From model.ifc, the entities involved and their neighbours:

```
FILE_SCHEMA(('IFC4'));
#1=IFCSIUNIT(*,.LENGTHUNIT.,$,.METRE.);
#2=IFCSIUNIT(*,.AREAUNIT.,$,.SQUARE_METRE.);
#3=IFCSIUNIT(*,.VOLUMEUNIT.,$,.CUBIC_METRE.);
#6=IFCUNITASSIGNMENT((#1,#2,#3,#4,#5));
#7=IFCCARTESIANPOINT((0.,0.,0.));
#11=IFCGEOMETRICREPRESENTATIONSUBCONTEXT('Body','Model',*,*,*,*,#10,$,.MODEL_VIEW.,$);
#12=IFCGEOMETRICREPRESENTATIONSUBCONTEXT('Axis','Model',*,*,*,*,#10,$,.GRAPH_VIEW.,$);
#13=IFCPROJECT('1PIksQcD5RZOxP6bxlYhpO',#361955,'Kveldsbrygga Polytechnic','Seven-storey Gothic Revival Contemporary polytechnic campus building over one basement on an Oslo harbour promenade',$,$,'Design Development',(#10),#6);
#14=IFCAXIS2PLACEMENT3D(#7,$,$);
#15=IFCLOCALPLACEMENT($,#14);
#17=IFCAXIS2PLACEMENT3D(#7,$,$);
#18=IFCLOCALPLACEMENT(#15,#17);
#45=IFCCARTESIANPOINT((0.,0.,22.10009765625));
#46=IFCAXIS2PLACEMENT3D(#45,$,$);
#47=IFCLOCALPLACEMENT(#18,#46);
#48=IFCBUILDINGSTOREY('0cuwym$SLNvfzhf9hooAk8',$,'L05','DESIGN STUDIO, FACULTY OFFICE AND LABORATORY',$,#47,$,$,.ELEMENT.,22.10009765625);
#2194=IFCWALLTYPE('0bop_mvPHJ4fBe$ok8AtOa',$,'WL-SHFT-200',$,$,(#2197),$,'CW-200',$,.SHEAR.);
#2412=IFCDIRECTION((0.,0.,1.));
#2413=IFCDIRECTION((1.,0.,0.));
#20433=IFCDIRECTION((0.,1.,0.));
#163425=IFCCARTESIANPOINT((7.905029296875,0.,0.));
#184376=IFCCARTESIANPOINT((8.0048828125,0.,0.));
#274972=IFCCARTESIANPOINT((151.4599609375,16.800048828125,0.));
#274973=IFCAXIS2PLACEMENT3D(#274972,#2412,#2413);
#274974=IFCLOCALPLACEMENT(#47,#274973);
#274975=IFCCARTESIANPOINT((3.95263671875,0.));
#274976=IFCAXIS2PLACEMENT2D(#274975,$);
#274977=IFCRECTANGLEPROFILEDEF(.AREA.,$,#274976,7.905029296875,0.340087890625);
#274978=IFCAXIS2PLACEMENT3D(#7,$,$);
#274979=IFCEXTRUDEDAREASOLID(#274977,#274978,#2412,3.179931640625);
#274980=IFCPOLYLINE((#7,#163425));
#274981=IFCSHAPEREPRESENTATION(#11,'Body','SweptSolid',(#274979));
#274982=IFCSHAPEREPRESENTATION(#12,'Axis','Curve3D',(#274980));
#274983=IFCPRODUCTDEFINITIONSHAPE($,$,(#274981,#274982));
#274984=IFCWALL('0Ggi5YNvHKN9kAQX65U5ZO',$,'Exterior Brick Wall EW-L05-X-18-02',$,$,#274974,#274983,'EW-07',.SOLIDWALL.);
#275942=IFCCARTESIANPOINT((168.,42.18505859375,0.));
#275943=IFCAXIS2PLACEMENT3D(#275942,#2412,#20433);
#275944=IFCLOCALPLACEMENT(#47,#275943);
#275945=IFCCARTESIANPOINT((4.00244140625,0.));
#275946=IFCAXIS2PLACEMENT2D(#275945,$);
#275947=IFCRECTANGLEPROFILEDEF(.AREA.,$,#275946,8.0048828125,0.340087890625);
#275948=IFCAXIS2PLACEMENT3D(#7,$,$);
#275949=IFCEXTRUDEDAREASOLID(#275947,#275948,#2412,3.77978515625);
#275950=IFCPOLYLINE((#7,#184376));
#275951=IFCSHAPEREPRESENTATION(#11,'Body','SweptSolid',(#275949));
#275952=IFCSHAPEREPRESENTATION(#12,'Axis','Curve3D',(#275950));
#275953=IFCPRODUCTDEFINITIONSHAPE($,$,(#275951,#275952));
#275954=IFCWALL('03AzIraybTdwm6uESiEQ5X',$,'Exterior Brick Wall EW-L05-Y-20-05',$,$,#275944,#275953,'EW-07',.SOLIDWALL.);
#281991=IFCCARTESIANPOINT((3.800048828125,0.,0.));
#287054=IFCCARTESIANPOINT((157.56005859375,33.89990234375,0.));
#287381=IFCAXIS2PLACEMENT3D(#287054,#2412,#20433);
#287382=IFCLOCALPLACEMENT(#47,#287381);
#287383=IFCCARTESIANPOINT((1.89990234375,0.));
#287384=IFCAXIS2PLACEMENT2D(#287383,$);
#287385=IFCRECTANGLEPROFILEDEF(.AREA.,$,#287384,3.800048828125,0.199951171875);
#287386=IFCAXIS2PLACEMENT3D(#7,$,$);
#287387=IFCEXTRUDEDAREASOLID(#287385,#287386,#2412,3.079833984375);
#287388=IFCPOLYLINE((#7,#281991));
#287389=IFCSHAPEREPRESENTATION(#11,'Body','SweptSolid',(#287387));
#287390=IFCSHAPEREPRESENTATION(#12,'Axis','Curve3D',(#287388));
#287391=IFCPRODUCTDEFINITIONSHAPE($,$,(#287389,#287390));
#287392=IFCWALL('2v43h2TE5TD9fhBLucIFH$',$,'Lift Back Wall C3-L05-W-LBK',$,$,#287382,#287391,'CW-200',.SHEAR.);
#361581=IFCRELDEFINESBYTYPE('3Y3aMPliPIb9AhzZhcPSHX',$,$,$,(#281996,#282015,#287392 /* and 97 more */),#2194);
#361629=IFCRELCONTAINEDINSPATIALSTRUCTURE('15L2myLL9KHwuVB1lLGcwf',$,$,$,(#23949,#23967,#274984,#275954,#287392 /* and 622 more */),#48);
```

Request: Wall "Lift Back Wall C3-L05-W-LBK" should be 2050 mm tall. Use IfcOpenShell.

```python
import ifcopenshell
import ifcopenshell.geom
import ifcopenshell.util.representation
import ifcopenshell.util.shape

model = ifcopenshell.open("model.ifc")
settings = ifcopenshell.geom.settings()


def volume(element):
    """Net volume in cubic metres, openings subtracted."""
    shape = ifcopenshell.geom.create_shape(settings, element)
    return ifcopenshell.util.shape.get_volume(shape.geometry)


wall = model.by_guid("2v43h2TE5TD9fhBLucIFH$")
before = volume(wall)

body = ifcopenshell.util.representation.get_representation(wall, "Model", "Body")
solid = body.Items[0]
old_height = solid.Depth
solid.Depth = 2.05
after = volume(wall)

print(f"height {old_height:g} -> {solid.Depth:g}, volume {before:.3f} -> {after:.3f} m3")

model.write("model_v2.ifc")
```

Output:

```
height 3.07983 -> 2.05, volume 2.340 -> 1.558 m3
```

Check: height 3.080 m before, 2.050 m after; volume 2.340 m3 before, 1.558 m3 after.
